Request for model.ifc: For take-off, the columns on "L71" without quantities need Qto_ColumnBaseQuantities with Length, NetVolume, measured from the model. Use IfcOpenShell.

First a look at what the model holds.

```python
import ifcopenshell
import ifcopenshell.util.element
import ifcopenshell.util.unit

model = ifcopenshell.open("model.ifc")
print(model.schema)
for unit_type in ("LENGTHUNIT", "AREAUNIT", "VOLUMEUNIT"):
    print(unit_type, ifcopenshell.util.unit.calculate_unit_scale(model, unit_type))
storey = next(s for s in model.by_type("IfcBuildingStorey") if s.Name == "L71")
columns = [e for e in ifcopenshell.util.element.get_decomposition(storey) if e.is_a("IfcColumn")]
for e in sorted(columns, key=lambda e: e.id()):
    print(e.id(), e.is_a(), e.Name, list(ifcopenshell.util.element.get_psets(e, qtos_only=True)), sep=" | ")
```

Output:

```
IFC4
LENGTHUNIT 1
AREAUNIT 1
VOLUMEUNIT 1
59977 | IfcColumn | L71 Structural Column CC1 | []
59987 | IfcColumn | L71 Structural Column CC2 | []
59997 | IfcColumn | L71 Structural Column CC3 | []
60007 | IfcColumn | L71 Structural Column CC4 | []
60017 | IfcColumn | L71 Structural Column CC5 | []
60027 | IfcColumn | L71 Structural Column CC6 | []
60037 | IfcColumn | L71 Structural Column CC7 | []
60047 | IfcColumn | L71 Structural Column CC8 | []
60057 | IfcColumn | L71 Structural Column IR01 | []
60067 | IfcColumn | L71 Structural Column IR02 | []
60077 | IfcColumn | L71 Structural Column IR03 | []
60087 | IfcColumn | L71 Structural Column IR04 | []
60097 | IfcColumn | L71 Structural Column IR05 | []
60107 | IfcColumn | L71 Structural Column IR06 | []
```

```python
import ifcopenshell
import ifcopenshell.api.pset
import ifcopenshell.geom
import ifcopenshell.util.element
import ifcopenshell.util.shape
import ifcopenshell.util.unit

model = ifcopenshell.open("model.ifc")
unit_scale = ifcopenshell.util.unit.calculate_unit_scale(model)
volume_scale = ifcopenshell.util.unit.calculate_unit_scale(model, "VOLUMEUNIT")
settings = ifcopenshell.geom.settings()

storey = next(s for s in model.by_type("IfcBuildingStorey") if s.Name == "L71")
columns = [e for e in ifcopenshell.util.element.get_decomposition(storey) if e.is_a("IfcColumn")]

for e in sorted(columns, key=lambda e: e.id()):
    if ifcopenshell.util.element.get_psets(e, qtos_only=True, should_inherit=False):
        continue
    # Geometry comes back in metres, in the element's own axes.
    shape = ifcopenshell.geom.create_shape(settings, e)
    values = {
        "Length": ifcopenshell.util.shape.get_z(shape.geometry) / unit_scale,
        "NetVolume": ifcopenshell.util.shape.get_volume(shape.geometry) / volume_scale,
    }
    qto = ifcopenshell.api.pset.add_qto(model, product=e, name="Qto_ColumnBaseQuantities")
    ifcopenshell.api.pset.edit_qto(model, qto=qto, properties=values)
    print(e.id(), {k: round(v, 3) for k, v in values.items()})

model.write("model_v2.ifc")
```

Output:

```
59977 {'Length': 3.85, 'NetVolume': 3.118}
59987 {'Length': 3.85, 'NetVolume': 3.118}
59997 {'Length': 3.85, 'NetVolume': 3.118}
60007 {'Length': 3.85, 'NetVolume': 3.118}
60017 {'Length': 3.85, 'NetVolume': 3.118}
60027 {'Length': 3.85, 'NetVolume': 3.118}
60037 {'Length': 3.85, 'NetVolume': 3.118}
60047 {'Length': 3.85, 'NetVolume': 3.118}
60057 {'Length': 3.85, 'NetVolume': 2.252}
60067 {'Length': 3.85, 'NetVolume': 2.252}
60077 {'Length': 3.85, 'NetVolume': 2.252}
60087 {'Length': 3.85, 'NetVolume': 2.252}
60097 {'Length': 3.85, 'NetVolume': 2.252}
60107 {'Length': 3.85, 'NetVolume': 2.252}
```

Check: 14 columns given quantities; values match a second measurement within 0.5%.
